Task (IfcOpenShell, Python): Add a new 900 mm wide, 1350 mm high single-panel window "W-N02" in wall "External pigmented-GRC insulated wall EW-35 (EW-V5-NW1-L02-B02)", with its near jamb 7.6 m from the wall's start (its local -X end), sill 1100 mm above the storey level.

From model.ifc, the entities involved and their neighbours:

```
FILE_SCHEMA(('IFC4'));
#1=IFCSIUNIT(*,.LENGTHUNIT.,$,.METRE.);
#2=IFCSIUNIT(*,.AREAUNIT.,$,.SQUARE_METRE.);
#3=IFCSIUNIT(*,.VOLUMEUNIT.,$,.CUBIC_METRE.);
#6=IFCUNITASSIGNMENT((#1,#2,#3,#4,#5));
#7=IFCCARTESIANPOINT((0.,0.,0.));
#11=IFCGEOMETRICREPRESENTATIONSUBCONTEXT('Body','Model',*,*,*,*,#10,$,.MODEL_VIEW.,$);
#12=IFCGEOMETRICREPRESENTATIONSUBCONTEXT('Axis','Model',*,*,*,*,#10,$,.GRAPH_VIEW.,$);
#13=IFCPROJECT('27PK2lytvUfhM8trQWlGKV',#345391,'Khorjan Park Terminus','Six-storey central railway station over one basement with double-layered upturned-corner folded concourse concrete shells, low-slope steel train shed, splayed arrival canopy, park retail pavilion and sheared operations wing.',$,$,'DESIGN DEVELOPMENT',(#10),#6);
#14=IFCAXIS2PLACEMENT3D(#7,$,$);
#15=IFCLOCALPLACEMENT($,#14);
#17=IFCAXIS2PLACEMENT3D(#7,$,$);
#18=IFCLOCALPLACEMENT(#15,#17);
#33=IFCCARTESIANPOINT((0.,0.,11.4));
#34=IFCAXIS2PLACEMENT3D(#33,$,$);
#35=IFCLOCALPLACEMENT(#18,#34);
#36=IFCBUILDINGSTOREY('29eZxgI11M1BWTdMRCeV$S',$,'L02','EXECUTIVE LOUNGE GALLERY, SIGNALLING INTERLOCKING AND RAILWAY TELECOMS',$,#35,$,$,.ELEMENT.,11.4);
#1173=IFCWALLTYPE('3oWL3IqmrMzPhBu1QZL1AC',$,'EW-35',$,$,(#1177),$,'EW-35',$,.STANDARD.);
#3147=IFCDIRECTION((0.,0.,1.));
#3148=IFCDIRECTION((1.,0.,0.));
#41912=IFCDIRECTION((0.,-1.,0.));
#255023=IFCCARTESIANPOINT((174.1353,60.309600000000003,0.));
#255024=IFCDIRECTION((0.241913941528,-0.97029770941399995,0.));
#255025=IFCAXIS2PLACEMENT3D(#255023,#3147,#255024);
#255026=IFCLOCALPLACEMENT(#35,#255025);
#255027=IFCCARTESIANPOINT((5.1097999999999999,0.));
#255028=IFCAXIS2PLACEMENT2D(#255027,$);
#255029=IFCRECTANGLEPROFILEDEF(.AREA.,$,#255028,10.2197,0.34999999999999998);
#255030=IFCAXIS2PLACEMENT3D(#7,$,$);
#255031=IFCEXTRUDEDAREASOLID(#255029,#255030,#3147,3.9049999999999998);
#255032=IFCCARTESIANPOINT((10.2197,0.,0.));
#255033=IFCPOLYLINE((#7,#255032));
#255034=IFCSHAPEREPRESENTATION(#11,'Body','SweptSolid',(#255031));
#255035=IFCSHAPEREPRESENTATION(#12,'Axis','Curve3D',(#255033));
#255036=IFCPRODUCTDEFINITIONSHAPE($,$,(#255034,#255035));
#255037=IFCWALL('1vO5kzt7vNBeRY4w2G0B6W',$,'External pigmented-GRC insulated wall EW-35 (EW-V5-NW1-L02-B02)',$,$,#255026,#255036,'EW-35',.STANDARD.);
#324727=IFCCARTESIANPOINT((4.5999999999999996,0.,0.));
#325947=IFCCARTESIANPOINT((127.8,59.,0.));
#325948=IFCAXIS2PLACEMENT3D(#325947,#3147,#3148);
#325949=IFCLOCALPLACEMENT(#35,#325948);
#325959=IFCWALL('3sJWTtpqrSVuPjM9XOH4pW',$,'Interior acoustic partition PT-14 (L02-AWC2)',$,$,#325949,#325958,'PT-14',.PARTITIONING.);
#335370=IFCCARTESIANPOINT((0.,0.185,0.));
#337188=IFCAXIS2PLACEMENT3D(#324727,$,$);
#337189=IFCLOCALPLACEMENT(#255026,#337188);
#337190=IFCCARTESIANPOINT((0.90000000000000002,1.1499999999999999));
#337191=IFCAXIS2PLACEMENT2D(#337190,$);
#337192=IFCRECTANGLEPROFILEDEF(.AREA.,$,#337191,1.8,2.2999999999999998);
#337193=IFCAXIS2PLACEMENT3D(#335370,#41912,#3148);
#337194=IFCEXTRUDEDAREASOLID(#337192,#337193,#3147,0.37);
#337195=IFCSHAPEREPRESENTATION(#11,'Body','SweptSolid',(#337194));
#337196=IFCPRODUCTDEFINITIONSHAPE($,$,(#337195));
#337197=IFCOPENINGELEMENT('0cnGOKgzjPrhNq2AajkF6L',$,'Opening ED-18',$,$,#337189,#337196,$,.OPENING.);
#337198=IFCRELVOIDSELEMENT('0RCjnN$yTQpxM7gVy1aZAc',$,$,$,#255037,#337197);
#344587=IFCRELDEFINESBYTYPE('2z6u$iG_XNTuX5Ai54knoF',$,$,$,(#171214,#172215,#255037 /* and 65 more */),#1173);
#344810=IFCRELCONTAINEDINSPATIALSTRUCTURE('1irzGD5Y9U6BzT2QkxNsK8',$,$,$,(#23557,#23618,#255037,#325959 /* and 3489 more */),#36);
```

```python
import numpy as np
import ifcopenshell
import ifcopenshell.api.feature
import ifcopenshell.api.geometry
import ifcopenshell.api.root
import ifcopenshell.api.spatial
import ifcopenshell.geom
import ifcopenshell.util.element
import ifcopenshell.util.placement
import ifcopenshell.util.representation
import ifcopenshell.util.shape
import ifcopenshell.util.unit

model = ifcopenshell.open("model.ifc")
unit_scale = ifcopenshell.util.unit.calculate_unit_scale(model)
settings = ifcopenshell.geom.settings()


def volume(element):
    """Net volume in cubic metres, openings subtracted."""
    shape = ifcopenshell.geom.create_shape(settings, element)
    return ifcopenshell.util.shape.get_volume(shape.geometry)


wall = model.by_guid("1vO5kzt7vNBeRY4w2G0B6W")
storey = ifcopenshell.util.element.get_container(wall, ifc_class="IfcBuildingStorey")
context = ifcopenshell.util.representation.get_context(model, "Model", "Body", "MODEL_VIEW")
before = volume(wall)

width, height, from_end, sill = 0.9, 1.35, 7.6, 1.1  # metres

# The wall runs along its own X axis, and the end named is its -X end.
wall_shape = ifcopenshell.geom.create_shape(settings, wall)
x, y, z = ifcopenshell.util.shape.get_vertices(wall_shape.geometry).T
start = x.min() + from_end
face, thickness = float(y.min()), float(y.max() - y.min())
wall_matrix = ifcopenshell.util.placement.get_local_placement(wall.ObjectPlacement)
level = ifcopenshell.util.placement.get_local_placement(storey.ObjectPlacement)[2, 3]


def in_wall(x, y):
    """Placement at x, y metres in the wall's axes, at sill height."""
    matrix = wall_matrix.copy()
    matrix[:, 3] = wall_matrix @ np.array([x / unit_scale, y / unit_scale, 0.0, 1.0])
    matrix[2, 3] = level + sill / unit_scale
    return matrix


# Opening: a box that overshoots both wall faces by 50 mm.
opening = ifcopenshell.api.root.create_entity(model, ifc_class="IfcOpeningElement", predefined_type="OPENING")
box = ifcopenshell.api.geometry.add_wall_representation(
    model, context=context, length=width, height=height, thickness=thickness + 0.1
)
ifcopenshell.api.geometry.assign_representation(model, product=opening, representation=box)
ifcopenshell.api.geometry.edit_object_placement(model, product=opening, matrix=in_wall(start, face - 0.05), is_si=False)
ifcopenshell.api.feature.add_feature(model, feature=opening, element=wall)

window = ifcopenshell.api.root.create_entity(model, ifc_class="IfcWindow", name="W-N02", predefined_type="WINDOW")
window.OverallWidth, window.OverallHeight = width / unit_scale, height / unit_scale
window.PartitioningType = "SINGLE_PANEL"
body = ifcopenshell.api.geometry.add_window_representation(
    model,
    context=context,
    overall_width=window.OverallWidth,
    overall_height=window.OverallHeight,
    partition_type="SINGLE_PANEL",
)
ifcopenshell.api.geometry.assign_representation(model, product=window, representation=body)
ifcopenshell.api.spatial.assign_container(model, products=[window], relating_structure=storey)
ifcopenshell.api.feature.add_filling(model, opening=opening, element=window)

# Centre the window in the wall's thickness.
ifcopenshell.api.geometry.edit_object_placement(model, product=window, matrix=in_wall(start, face), is_si=False)
window_shape = ifcopenshell.geom.create_shape(settings, window)
depth = ifcopenshell.util.shape.get_vertices(window_shape.geometry)[:, 1]
offset = face + thickness / 2 - (depth.min() + depth.max()) / 2
ifcopenshell.api.geometry.edit_object_placement(model, product=window, matrix=in_wall(start, offset), is_si=False)

after = volume(wall)

print(f"wall volume {before:.3f} -> {after:.3f} m3")

model.write("model_edited.ifc")
```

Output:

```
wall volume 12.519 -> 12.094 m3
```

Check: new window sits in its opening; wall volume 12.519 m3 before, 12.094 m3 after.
